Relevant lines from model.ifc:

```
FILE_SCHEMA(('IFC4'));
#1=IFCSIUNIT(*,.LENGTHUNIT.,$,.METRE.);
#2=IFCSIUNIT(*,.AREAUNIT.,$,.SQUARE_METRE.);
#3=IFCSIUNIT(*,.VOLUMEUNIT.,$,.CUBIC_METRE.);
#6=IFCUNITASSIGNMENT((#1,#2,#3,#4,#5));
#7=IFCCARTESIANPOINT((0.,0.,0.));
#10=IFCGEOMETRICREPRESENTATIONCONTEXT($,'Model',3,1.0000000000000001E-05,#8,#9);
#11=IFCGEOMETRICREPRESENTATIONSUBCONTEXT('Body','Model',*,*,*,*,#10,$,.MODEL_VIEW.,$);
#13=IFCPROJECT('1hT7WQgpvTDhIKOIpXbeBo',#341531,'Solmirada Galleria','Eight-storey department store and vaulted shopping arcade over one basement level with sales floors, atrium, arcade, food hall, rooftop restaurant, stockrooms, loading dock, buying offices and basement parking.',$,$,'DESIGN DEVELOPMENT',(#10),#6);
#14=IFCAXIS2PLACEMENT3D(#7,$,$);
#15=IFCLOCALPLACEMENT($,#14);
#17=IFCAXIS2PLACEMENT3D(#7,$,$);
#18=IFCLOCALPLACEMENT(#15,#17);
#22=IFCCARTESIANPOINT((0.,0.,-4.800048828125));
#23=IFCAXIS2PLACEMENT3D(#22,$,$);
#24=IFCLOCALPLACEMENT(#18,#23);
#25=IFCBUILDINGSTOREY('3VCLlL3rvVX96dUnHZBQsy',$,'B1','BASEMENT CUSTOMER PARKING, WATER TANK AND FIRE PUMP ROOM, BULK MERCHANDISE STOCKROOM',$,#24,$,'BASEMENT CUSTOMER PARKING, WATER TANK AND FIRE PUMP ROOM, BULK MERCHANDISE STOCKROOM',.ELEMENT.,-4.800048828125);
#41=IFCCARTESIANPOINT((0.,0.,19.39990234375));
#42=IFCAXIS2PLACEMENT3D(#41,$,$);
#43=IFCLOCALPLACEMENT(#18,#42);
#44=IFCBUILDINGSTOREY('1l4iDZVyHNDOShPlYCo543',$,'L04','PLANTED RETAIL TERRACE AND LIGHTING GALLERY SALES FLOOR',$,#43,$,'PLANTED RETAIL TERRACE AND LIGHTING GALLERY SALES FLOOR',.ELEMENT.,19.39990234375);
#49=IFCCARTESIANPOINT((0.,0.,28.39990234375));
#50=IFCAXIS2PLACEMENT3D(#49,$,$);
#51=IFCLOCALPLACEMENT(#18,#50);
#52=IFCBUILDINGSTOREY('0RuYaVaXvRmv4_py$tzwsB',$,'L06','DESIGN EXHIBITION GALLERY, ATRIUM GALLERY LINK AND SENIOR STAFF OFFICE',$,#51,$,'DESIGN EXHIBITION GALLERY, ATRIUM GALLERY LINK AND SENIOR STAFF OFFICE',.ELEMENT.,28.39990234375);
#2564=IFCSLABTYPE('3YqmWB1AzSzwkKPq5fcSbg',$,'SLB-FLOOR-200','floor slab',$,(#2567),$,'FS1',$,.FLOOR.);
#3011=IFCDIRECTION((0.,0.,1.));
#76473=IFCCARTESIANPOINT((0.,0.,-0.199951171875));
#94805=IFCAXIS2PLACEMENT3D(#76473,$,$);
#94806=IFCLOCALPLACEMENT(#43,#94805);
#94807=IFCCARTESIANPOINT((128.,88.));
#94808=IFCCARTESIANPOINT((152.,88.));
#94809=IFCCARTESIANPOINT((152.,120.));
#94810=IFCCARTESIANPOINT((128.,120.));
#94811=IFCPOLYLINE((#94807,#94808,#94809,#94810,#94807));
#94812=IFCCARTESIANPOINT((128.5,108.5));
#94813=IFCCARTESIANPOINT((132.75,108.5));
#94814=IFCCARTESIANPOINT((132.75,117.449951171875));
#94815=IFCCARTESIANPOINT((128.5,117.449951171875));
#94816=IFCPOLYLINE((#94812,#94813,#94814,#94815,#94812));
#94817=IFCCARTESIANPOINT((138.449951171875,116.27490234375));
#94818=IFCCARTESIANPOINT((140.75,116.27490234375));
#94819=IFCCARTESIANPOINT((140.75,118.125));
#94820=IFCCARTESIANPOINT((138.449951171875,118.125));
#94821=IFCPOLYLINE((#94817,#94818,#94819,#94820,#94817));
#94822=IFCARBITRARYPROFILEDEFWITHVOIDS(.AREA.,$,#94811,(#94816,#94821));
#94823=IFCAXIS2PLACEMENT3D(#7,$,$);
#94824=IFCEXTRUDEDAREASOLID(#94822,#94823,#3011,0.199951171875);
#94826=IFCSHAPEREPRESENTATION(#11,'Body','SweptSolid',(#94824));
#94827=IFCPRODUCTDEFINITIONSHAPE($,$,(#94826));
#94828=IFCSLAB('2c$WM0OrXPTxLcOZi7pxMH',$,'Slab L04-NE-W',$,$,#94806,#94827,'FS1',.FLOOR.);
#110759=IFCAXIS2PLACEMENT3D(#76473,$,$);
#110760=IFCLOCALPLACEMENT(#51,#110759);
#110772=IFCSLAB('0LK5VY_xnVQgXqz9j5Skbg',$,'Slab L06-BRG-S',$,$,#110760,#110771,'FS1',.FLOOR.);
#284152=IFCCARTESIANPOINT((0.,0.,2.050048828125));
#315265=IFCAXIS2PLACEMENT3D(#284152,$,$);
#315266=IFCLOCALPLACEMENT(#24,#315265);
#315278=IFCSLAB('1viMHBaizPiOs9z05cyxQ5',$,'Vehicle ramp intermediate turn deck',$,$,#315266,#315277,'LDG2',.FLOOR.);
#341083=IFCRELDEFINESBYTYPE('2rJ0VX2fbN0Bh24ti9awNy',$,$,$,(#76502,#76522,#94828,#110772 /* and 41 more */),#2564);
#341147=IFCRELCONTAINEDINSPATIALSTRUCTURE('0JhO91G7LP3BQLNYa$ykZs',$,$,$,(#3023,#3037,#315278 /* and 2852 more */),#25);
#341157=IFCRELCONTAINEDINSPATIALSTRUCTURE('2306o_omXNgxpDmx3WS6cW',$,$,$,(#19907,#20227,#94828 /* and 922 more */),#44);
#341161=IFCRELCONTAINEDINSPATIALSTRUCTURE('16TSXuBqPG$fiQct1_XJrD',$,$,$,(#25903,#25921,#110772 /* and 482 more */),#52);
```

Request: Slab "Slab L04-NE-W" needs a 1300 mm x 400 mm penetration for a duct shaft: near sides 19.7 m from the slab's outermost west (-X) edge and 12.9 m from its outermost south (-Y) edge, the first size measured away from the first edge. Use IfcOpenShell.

```python
import numpy as np
import ifcopenshell
import ifcopenshell.api.feature
import ifcopenshell.api.geometry
import ifcopenshell.api.root
import ifcopenshell.geom
import ifcopenshell.util.placement
import ifcopenshell.util.representation
import ifcopenshell.util.shape
import ifcopenshell.util.unit

model = ifcopenshell.open("model.ifc")
unit_scale = ifcopenshell.util.unit.calculate_unit_scale(model)
settings = ifcopenshell.geom.settings()


def volume(element):
    """Net volume in cubic metres, openings subtracted."""
    shape = ifcopenshell.geom.create_shape(settings, element)
    return ifcopenshell.util.shape.get_volume(shape.geometry)


slab = model.by_guid("2c$WM0OrXPTxLcOZi7pxMH")
before = volume(slab)

# Extent in the slab's own axes, in metres. The edges named are its -X and -Y sides.
slab_shape = ifcopenshell.geom.create_shape(settings, slab)
vertices = ifcopenshell.util.shape.get_vertices(slab_shape.geometry)
x_min, y_min, bottom = vertices.min(axis=0)
top = vertices[:, 2].max()

opening = ifcopenshell.api.root.create_entity(model, ifc_class="IfcOpeningElement", name="Duct shaft opening", predefined_type="OPENING")
context = ifcopenshell.util.representation.get_context(model, "Model", "Body", "MODEL_VIEW")
width, depth = 1.3, 0.4
outline = [(0.0, 0.0), (width, 0.0), (width, depth), (0.0, depth), (0.0, 0.0)]
# Overshoot both faces by 50 mm so the cut is clean.
shape = ifcopenshell.api.geometry.add_slab_representation(
    model, context=context, depth=top - bottom + 0.1, polyline=outline
)
ifcopenshell.api.geometry.assign_representation(model, product=opening, representation=shape)

matrix = ifcopenshell.util.placement.get_local_placement(slab.ObjectPlacement)
matrix[:, 3] = matrix @ np.append(np.array([x_min + 19.7, y_min + 12.9, bottom - 0.05]) / unit_scale, 1.0)
ifcopenshell.api.geometry.edit_object_placement(model, product=opening, matrix=matrix, is_si=False)
ifcopenshell.api.feature.add_feature(model, feature=opening, element=slab)

after = volume(slab)

print(f"slab volume {before:.3f} -> {after:.3f} m3")

model.write("model_edited.ifc")
```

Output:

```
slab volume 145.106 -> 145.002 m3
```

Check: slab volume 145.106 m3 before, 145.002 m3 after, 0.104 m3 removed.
